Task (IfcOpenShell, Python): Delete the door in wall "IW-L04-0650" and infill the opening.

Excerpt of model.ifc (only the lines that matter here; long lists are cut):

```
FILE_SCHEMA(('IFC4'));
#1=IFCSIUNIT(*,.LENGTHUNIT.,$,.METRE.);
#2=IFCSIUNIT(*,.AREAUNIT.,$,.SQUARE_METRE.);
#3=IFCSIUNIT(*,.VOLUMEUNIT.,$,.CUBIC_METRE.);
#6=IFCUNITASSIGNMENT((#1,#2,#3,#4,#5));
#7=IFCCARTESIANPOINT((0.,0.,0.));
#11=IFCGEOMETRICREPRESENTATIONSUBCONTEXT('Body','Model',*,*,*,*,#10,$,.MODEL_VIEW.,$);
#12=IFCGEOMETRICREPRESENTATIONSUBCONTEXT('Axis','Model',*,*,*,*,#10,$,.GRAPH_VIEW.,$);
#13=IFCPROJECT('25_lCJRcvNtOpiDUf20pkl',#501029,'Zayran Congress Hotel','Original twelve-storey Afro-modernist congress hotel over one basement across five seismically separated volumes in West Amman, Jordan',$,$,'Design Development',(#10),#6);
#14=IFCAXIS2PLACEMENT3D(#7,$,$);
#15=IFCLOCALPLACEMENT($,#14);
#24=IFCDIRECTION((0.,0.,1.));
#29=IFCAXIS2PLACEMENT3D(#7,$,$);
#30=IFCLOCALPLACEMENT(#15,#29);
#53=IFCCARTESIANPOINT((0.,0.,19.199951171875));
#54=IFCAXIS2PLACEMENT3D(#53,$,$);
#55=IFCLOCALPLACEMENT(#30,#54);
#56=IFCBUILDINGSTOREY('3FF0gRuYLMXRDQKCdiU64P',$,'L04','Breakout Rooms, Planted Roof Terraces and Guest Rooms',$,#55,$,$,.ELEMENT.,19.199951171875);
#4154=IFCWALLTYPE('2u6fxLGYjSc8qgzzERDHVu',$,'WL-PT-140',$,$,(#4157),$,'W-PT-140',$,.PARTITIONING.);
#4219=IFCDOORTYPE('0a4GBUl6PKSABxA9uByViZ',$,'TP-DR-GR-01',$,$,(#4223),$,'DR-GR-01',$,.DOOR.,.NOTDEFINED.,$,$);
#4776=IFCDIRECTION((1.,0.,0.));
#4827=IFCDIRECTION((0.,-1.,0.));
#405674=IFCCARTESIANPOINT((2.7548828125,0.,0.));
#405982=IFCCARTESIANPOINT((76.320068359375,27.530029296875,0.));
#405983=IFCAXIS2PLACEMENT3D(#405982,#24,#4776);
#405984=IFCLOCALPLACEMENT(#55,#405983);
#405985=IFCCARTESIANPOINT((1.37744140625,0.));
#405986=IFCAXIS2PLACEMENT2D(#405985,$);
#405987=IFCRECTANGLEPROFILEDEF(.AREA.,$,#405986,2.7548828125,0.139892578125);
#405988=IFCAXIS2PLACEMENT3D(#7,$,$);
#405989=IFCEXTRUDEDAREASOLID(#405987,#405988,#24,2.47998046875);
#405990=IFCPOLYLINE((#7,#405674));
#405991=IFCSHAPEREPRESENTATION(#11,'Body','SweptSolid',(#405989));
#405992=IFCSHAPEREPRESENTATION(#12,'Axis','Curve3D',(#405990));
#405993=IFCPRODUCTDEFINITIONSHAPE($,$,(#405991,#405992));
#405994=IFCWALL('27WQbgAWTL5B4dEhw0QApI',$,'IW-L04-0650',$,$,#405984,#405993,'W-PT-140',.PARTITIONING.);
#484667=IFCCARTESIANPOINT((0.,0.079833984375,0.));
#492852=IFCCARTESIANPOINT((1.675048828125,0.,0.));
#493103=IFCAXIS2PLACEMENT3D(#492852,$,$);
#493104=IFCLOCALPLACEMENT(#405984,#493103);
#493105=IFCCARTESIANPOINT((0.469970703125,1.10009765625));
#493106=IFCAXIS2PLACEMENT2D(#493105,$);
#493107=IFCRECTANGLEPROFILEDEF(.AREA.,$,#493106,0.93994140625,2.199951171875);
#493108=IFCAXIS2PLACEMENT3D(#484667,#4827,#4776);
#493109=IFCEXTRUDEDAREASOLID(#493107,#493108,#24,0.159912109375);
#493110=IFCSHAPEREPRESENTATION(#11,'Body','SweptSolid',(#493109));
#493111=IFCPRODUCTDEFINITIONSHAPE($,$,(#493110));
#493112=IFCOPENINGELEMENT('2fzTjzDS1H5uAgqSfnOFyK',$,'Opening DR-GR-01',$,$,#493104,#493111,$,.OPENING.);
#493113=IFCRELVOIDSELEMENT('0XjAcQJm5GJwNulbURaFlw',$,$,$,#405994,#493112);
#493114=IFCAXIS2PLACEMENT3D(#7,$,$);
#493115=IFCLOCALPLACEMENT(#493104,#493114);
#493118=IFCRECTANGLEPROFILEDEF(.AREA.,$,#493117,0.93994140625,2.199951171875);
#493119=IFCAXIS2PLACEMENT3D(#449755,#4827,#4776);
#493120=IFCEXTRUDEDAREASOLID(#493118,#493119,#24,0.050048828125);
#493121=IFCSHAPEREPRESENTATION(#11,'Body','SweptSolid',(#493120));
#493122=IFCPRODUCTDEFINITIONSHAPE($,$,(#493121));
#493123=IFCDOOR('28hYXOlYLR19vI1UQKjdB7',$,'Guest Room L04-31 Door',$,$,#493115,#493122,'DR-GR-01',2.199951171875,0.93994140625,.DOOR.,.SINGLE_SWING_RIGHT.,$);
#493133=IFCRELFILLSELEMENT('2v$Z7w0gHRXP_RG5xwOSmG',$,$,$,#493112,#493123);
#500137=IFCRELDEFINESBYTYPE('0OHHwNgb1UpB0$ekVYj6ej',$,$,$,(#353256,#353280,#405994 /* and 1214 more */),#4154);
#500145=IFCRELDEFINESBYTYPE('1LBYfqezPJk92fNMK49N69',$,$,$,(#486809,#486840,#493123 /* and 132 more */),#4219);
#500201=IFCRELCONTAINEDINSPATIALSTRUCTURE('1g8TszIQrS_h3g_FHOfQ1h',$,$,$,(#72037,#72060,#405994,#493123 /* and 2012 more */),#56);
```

```python
import ifcopenshell
import ifcopenshell.api.feature
import ifcopenshell.api.root
import ifcopenshell.geom
import ifcopenshell.util.shape

model = ifcopenshell.open("model.ifc")
settings = ifcopenshell.geom.settings()


def volume(element):
    """Net volume in cubic metres, openings subtracted."""
    shape = ifcopenshell.geom.create_shape(settings, element)
    return ifcopenshell.util.shape.get_volume(shape.geometry)


door = model.by_guid("28hYXOlYLR19vI1UQKjdB7")
opening = door.FillsVoids[0].RelatingOpeningElement
wall = opening.VoidsElements[0].RelatingBuildingElement
before = volume(wall)

ifcopenshell.api.root.remove_product(model, product=door)
ifcopenshell.api.feature.remove_feature(model, feature=opening)

after = volume(wall)

print(f"wall volume {before:.3f} -> {after:.3f} m3")

model.write("model_v2.ifc")
```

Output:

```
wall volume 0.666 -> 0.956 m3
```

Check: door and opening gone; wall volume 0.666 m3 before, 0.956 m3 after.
